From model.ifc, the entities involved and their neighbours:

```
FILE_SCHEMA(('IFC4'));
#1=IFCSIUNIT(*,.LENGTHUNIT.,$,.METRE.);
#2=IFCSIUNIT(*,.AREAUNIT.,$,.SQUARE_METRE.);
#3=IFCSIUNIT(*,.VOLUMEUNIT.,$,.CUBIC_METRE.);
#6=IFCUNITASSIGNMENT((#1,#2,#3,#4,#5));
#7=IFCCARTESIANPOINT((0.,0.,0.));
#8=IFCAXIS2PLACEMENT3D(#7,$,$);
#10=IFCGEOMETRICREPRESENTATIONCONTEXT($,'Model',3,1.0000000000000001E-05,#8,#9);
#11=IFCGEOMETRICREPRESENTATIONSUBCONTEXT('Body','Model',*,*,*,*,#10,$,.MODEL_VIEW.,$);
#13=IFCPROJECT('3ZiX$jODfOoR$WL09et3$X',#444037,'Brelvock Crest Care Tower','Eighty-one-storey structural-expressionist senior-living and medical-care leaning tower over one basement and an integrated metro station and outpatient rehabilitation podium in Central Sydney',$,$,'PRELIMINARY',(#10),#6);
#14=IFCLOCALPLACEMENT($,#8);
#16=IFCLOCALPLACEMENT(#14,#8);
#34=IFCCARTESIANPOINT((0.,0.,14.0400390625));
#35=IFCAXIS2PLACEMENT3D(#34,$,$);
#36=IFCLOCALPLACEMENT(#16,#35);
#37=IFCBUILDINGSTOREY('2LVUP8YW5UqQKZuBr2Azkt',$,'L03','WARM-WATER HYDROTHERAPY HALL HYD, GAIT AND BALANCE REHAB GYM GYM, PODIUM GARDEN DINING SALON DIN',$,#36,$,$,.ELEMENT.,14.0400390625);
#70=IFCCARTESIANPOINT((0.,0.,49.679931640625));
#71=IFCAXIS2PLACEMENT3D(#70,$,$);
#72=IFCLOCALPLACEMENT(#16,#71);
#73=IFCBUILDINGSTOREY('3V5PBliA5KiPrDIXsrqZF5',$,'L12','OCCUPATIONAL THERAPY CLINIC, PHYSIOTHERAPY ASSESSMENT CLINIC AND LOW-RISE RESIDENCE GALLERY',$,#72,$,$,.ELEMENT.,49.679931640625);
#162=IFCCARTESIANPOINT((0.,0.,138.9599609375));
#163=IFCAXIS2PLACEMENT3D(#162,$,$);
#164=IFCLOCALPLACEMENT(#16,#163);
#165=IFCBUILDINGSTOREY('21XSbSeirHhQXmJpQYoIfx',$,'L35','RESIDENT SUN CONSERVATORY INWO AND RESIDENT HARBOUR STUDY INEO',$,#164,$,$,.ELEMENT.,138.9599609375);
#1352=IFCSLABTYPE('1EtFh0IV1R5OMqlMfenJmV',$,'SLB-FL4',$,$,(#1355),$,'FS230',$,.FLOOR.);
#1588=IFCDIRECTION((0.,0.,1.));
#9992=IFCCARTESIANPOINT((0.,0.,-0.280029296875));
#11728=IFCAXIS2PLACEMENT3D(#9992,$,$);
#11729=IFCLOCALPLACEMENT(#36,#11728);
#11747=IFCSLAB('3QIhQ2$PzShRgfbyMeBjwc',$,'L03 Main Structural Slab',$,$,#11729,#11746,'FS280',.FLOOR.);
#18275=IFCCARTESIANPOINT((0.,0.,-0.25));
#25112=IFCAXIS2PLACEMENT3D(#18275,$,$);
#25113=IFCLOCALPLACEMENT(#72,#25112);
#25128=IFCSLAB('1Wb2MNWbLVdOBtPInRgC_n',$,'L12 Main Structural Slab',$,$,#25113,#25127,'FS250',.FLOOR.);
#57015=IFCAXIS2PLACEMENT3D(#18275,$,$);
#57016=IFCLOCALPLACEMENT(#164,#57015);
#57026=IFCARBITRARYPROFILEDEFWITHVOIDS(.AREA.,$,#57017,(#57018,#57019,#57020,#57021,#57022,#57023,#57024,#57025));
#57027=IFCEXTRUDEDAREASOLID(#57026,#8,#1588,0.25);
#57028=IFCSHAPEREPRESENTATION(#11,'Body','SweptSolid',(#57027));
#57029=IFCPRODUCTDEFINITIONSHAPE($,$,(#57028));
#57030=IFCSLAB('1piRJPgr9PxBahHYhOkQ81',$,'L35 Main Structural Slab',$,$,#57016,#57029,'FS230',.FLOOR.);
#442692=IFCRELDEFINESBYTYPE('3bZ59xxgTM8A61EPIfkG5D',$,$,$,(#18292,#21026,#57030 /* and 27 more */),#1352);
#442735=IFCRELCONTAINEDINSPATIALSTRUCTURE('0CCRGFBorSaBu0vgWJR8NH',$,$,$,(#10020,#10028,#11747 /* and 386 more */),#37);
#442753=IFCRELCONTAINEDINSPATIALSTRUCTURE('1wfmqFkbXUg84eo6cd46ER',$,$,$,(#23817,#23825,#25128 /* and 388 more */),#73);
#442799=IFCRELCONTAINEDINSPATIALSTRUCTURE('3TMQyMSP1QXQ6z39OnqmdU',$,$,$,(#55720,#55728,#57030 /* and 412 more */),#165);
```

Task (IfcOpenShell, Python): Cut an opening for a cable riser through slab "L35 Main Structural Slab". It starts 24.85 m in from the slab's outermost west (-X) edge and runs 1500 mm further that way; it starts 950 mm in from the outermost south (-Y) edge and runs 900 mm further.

```python
import numpy as np
import ifcopenshell
import ifcopenshell.api.feature
import ifcopenshell.api.geometry
import ifcopenshell.api.root
import ifcopenshell.geom
import ifcopenshell.util.placement
import ifcopenshell.util.representation
import ifcopenshell.util.shape
import ifcopenshell.util.unit

model = ifcopenshell.open("model.ifc")
unit_scale = ifcopenshell.util.unit.calculate_unit_scale(model)
settings = ifcopenshell.geom.settings()


def volume(element):
    """Net volume in cubic metres, openings subtracted."""
    shape = ifcopenshell.geom.create_shape(settings, element)
    return ifcopenshell.util.shape.get_volume(shape.geometry)


slab = model.by_guid("1piRJPgr9PxBahHYhOkQ81")
before = volume(slab)

# Extent in the slab's own axes, in metres. The edges named are its -X and -Y sides.
slab_shape = ifcopenshell.geom.create_shape(settings, slab)
vertices = ifcopenshell.util.shape.get_vertices(slab_shape.geometry)
x_min, y_min, bottom = vertices.min(axis=0)
top = vertices[:, 2].max()

opening = ifcopenshell.api.root.create_entity(model, ifc_class="IfcOpeningElement", name="Cable riser opening", predefined_type="OPENING")
context = ifcopenshell.util.representation.get_context(model, "Model", "Body", "MODEL_VIEW")
width, depth = 1.5, 0.9
outline = [(0.0, 0.0), (width, 0.0), (width, depth), (0.0, depth), (0.0, 0.0)]
# Overshoot both faces by 50 mm so the cut is clean.
shape = ifcopenshell.api.geometry.add_slab_representation(
    model, context=context, depth=top - bottom + 0.1, polyline=outline
)
ifcopenshell.api.geometry.assign_representation(model, product=opening, representation=shape)

matrix = ifcopenshell.util.placement.get_local_placement(slab.ObjectPlacement)
matrix[:, 3] = matrix @ np.append(np.array([x_min + 24.85, y_min + 0.95, bottom - 0.05]) / unit_scale, 1.0)
ifcopenshell.api.geometry.edit_object_placement(model, product=opening, matrix=matrix, is_si=False)
ifcopenshell.api.feature.add_feature(model, feature=opening, element=slab)

after = volume(slab)

print(f"slab volume {before:.3f} -> {after:.3f} m3")

model.write("model_v2.ifc")
```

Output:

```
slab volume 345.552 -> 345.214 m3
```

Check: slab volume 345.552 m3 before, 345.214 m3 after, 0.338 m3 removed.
